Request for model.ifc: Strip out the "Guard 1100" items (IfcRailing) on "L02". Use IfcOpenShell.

First a look at what the model holds.

```python
import ifcopenshell
import ifcopenshell.util.element

model = ifcopenshell.open("model.ifc")
print(model.schema)
storey = next(s for s in model.by_type("IfcBuildingStorey") if s.Name == "L02")
railings = [e for e in ifcopenshell.util.element.get_decomposition(storey) if e.is_a("IfcRailing")]
seen = {}
for e in railings:
    element_type = ifcopenshell.util.element.get_type(e)
    name = element_type.Name if element_type not in (None, e) else None
    seen[name] = seen.get(name, 0) + 1
for name, count in sorted(seen.items(), key=str):
    print(count, "x", name)
```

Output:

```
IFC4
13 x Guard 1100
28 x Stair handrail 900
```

```python
import ifcopenshell
import ifcopenshell.api.root
import ifcopenshell.util.element

model = ifcopenshell.open("model.ifc")

storey = next(s for s in model.by_type("IfcBuildingStorey") if s.Name == "L02")
railings = [e for e in ifcopenshell.util.element.get_decomposition(storey) if e.is_a("IfcRailing")]
targets = [e for e in railings if (t := ifcopenshell.util.element.get_type(e)) not in (None, e) and t.Name == "Guard 1100"]

for e in targets:
    ifcopenshell.api.root.remove_product(model, product=e)
print(len(targets), "removed")

model.write("model_rev.ifc")
```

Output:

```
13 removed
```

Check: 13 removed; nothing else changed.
